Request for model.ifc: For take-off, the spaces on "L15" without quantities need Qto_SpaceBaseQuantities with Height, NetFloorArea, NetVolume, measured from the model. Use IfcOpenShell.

First a look at what the model holds.

```python
import ifcopenshell
import ifcopenshell.util.element
import ifcopenshell.util.unit

model = ifcopenshell.open("model.ifc")
print(model.schema)
for unit_type in ("LENGTHUNIT", "AREAUNIT", "VOLUMEUNIT"):
    print(unit_type, ifcopenshell.util.unit.calculate_unit_scale(model, unit_type))
storey = next(s for s in model.by_type("IfcBuildingStorey") if s.Name == "L15")
spaces = [e for e in ifcopenshell.util.element.get_decomposition(storey) if e.is_a("IfcSpace")]
for e in sorted(spaces, key=lambda e: e.id()):
    print(e.id(), e.is_a(), e.Name, list(ifcopenshell.util.element.get_psets(e, qtos_only=True)), sep=" | ")
```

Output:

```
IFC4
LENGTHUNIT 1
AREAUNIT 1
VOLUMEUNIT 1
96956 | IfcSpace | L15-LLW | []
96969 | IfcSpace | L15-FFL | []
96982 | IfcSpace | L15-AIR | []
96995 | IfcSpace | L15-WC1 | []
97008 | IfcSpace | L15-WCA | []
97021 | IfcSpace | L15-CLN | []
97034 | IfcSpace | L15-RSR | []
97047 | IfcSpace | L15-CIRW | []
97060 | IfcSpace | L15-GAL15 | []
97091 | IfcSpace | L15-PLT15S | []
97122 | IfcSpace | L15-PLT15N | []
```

```python
import ifcopenshell
import ifcopenshell.api.pset
import ifcopenshell.geom
import ifcopenshell.util.element
import ifcopenshell.util.shape
import ifcopenshell.util.unit

model = ifcopenshell.open("model.ifc")
unit_scale = ifcopenshell.util.unit.calculate_unit_scale(model)
area_scale = ifcopenshell.util.unit.calculate_unit_scale(model, "AREAUNIT")
volume_scale = ifcopenshell.util.unit.calculate_unit_scale(model, "VOLUMEUNIT")
settings = ifcopenshell.geom.settings()

storey = next(s for s in model.by_type("IfcBuildingStorey") if s.Name == "L15")
spaces = [e for e in ifcopenshell.util.element.get_decomposition(storey) if e.is_a("IfcSpace")]

for e in sorted(spaces, key=lambda e: e.id()):
    if ifcopenshell.util.element.get_psets(e, qtos_only=True, should_inherit=False):
        continue
    # Geometry comes back in metres, in the element's own axes.
    shape = ifcopenshell.geom.create_shape(settings, e)
    values = {
        "Height": ifcopenshell.util.shape.get_z(shape.geometry) / unit_scale,
        "NetFloorArea": ifcopenshell.util.shape.get_footprint_area(shape.geometry) / area_scale,
        "NetVolume": ifcopenshell.util.shape.get_volume(shape.geometry) / volume_scale,
    }
    qto = ifcopenshell.api.pset.add_qto(model, product=e, name="Qto_SpaceBaseQuantities")
    ifcopenshell.api.pset.edit_qto(model, qto=qto, properties=values)
    print(e.id(), {k: round(v, 3) for k, v in values.items()})

model.write("model_v2.ifc")
```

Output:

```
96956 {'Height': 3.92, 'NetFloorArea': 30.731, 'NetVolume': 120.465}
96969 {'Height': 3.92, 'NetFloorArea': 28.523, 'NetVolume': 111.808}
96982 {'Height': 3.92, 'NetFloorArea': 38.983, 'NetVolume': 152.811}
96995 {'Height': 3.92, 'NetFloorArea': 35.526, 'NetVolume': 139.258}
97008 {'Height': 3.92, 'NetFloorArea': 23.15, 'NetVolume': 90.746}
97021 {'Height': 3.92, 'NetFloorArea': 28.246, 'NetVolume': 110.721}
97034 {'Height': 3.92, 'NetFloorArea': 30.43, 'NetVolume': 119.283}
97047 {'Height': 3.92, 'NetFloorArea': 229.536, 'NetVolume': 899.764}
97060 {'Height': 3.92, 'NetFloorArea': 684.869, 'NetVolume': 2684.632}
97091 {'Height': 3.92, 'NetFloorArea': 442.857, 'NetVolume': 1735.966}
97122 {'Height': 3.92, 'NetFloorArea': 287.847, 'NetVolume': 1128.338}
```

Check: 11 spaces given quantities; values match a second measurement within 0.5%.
